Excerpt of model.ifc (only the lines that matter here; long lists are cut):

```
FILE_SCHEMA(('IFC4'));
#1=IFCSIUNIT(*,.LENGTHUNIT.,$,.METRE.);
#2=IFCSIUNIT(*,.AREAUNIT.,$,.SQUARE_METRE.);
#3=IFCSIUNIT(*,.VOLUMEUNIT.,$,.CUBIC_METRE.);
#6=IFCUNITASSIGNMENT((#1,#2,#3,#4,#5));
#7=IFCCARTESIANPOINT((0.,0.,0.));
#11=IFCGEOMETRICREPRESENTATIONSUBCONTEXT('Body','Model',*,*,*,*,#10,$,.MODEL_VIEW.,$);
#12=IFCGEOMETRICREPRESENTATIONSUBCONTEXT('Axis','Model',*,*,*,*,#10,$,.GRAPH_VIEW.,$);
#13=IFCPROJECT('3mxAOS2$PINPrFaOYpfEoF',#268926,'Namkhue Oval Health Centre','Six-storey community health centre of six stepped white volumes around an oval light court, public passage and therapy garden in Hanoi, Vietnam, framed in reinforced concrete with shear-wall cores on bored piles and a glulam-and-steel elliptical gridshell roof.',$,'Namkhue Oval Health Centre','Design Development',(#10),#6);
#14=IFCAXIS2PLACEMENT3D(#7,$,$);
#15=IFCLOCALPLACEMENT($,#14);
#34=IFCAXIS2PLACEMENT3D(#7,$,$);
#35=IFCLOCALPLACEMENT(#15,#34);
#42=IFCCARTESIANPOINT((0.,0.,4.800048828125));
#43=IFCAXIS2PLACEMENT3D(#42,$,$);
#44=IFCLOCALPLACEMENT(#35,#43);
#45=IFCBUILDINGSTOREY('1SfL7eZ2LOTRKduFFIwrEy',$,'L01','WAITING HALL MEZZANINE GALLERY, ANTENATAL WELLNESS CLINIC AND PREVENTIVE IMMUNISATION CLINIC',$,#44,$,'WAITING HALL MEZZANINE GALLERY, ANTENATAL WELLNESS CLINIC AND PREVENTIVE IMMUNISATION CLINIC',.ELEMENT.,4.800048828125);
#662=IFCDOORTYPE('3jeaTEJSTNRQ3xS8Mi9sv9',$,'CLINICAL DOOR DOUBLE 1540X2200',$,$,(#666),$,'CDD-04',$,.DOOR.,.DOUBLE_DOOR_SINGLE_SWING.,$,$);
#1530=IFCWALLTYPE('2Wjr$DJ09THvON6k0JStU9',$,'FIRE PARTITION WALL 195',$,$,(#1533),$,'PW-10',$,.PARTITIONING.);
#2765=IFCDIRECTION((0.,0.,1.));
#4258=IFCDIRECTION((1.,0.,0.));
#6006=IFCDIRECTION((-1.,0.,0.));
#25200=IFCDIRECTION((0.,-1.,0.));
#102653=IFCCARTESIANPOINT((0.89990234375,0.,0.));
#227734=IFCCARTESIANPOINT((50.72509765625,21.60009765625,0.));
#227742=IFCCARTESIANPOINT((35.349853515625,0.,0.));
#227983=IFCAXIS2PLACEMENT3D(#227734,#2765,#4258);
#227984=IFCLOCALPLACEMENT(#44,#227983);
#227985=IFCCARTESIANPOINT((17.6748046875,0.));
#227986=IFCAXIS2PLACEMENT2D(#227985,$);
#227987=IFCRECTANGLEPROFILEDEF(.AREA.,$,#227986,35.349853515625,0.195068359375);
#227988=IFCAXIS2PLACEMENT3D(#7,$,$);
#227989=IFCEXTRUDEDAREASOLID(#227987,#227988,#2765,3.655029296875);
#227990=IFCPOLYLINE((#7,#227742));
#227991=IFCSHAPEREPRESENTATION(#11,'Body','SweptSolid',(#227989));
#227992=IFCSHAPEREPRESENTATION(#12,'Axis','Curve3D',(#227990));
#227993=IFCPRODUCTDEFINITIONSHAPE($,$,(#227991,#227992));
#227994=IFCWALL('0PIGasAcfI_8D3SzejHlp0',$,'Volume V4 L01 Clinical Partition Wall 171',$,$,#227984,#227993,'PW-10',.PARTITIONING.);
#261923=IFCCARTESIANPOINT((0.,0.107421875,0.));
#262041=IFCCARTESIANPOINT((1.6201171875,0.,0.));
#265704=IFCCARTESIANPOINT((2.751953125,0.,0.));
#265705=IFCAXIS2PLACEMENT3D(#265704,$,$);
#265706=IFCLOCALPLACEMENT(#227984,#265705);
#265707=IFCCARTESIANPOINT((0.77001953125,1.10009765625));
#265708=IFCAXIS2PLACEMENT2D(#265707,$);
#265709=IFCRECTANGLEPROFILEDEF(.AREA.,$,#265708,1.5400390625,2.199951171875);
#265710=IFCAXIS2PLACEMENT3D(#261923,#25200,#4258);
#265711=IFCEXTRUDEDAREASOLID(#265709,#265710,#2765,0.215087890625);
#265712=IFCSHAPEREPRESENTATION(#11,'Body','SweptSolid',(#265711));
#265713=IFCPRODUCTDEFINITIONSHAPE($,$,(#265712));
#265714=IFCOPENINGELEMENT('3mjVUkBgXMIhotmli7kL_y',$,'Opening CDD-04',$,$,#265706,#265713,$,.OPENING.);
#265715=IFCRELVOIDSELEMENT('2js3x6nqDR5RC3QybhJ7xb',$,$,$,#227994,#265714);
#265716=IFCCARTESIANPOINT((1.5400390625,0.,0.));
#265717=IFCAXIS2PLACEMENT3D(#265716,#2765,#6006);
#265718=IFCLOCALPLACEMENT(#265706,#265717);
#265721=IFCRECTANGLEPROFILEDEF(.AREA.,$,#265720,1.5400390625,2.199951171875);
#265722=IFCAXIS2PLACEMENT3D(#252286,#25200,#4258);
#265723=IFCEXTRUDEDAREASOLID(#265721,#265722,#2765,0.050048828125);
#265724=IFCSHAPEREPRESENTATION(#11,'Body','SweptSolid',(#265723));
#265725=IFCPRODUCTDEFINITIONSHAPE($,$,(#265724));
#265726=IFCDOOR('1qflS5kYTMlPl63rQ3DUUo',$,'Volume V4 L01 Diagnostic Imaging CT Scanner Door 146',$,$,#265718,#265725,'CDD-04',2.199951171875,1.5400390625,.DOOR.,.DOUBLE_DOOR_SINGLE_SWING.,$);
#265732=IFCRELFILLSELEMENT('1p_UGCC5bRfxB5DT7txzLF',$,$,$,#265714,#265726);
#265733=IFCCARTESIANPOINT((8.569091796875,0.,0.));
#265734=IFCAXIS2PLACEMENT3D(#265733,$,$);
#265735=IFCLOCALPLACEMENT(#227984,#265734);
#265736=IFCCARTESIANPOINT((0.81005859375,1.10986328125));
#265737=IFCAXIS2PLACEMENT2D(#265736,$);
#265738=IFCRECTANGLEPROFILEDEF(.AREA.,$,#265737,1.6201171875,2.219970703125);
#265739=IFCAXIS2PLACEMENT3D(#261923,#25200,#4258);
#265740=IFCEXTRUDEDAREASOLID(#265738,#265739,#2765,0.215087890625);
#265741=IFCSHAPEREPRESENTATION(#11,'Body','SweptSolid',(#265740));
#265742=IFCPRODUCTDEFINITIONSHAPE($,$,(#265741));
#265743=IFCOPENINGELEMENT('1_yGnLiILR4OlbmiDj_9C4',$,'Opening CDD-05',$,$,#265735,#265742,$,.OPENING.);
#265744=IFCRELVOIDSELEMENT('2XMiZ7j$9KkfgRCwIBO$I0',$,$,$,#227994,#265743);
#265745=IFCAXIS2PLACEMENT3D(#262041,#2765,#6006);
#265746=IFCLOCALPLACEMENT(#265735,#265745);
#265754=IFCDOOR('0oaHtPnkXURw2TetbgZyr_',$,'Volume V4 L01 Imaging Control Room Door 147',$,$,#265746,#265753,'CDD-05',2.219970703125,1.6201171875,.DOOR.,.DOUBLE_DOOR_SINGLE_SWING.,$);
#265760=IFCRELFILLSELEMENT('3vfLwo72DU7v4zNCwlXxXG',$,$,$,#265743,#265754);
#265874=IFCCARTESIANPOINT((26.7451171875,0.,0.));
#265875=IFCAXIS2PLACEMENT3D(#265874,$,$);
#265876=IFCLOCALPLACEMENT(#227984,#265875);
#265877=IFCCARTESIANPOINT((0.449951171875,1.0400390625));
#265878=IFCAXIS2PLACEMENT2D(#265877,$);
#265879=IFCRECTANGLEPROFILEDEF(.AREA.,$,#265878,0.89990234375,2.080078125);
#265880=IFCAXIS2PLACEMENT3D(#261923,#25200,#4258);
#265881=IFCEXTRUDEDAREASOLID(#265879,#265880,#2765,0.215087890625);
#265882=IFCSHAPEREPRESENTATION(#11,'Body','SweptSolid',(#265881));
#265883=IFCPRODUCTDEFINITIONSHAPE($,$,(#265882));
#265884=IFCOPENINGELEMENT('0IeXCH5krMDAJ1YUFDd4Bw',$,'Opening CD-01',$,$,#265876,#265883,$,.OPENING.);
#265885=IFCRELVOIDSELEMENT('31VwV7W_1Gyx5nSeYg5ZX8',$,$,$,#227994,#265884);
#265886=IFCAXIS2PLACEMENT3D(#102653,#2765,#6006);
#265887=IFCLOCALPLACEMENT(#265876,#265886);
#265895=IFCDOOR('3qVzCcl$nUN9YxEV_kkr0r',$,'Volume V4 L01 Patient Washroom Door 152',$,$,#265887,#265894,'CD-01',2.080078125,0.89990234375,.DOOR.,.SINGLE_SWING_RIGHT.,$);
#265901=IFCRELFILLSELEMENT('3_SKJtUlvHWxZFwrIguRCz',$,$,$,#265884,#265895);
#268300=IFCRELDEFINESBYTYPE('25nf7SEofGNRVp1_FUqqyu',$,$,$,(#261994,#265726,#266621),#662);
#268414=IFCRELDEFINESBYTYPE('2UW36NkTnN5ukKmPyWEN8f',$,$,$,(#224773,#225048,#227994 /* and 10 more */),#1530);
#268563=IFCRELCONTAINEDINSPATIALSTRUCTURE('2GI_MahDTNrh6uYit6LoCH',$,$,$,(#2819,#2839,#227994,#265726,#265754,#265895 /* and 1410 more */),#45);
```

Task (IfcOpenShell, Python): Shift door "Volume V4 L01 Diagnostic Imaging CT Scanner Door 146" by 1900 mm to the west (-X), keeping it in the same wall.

```python
import ifcopenshell
import ifcopenshell.api.geometry
import ifcopenshell.util.placement
import ifcopenshell.util.unit

model = ifcopenshell.open("model.ifc")
unit_scale = ifcopenshell.util.unit.calculate_unit_scale(model)

door = model.by_guid("1qflS5kYTMlPl63rQ3DUUo")
opening = door.FillsVoids[0].RelatingOpeningElement
wall = opening.VoidsElements[0].RelatingBuildingElement

wall_matrix = ifcopenshell.util.placement.get_local_placement(wall.ObjectPlacement)
shift = wall_matrix[:3, 0] * -1.9 / unit_scale
before = ifcopenshell.util.placement.get_local_placement(door.ObjectPlacement)[:3, 3].copy()

# The door is placed relative to its opening, so it follows when the opening moves.
matrix = ifcopenshell.util.placement.get_local_placement(opening.ObjectPlacement)
matrix[:3, 3] += shift
ifcopenshell.api.geometry.edit_object_placement(
    model, product=opening, matrix=matrix, is_si=False, should_transform_children=True
)

after = ifcopenshell.util.placement.get_local_placement(door.ObjectPlacement)[:3, 3]
print("door moved by", (after - before).round(3) + 0.0)

model.write("model_v2.ifc")
```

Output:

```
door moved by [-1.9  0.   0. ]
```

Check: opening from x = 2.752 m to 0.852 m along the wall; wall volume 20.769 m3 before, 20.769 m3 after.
